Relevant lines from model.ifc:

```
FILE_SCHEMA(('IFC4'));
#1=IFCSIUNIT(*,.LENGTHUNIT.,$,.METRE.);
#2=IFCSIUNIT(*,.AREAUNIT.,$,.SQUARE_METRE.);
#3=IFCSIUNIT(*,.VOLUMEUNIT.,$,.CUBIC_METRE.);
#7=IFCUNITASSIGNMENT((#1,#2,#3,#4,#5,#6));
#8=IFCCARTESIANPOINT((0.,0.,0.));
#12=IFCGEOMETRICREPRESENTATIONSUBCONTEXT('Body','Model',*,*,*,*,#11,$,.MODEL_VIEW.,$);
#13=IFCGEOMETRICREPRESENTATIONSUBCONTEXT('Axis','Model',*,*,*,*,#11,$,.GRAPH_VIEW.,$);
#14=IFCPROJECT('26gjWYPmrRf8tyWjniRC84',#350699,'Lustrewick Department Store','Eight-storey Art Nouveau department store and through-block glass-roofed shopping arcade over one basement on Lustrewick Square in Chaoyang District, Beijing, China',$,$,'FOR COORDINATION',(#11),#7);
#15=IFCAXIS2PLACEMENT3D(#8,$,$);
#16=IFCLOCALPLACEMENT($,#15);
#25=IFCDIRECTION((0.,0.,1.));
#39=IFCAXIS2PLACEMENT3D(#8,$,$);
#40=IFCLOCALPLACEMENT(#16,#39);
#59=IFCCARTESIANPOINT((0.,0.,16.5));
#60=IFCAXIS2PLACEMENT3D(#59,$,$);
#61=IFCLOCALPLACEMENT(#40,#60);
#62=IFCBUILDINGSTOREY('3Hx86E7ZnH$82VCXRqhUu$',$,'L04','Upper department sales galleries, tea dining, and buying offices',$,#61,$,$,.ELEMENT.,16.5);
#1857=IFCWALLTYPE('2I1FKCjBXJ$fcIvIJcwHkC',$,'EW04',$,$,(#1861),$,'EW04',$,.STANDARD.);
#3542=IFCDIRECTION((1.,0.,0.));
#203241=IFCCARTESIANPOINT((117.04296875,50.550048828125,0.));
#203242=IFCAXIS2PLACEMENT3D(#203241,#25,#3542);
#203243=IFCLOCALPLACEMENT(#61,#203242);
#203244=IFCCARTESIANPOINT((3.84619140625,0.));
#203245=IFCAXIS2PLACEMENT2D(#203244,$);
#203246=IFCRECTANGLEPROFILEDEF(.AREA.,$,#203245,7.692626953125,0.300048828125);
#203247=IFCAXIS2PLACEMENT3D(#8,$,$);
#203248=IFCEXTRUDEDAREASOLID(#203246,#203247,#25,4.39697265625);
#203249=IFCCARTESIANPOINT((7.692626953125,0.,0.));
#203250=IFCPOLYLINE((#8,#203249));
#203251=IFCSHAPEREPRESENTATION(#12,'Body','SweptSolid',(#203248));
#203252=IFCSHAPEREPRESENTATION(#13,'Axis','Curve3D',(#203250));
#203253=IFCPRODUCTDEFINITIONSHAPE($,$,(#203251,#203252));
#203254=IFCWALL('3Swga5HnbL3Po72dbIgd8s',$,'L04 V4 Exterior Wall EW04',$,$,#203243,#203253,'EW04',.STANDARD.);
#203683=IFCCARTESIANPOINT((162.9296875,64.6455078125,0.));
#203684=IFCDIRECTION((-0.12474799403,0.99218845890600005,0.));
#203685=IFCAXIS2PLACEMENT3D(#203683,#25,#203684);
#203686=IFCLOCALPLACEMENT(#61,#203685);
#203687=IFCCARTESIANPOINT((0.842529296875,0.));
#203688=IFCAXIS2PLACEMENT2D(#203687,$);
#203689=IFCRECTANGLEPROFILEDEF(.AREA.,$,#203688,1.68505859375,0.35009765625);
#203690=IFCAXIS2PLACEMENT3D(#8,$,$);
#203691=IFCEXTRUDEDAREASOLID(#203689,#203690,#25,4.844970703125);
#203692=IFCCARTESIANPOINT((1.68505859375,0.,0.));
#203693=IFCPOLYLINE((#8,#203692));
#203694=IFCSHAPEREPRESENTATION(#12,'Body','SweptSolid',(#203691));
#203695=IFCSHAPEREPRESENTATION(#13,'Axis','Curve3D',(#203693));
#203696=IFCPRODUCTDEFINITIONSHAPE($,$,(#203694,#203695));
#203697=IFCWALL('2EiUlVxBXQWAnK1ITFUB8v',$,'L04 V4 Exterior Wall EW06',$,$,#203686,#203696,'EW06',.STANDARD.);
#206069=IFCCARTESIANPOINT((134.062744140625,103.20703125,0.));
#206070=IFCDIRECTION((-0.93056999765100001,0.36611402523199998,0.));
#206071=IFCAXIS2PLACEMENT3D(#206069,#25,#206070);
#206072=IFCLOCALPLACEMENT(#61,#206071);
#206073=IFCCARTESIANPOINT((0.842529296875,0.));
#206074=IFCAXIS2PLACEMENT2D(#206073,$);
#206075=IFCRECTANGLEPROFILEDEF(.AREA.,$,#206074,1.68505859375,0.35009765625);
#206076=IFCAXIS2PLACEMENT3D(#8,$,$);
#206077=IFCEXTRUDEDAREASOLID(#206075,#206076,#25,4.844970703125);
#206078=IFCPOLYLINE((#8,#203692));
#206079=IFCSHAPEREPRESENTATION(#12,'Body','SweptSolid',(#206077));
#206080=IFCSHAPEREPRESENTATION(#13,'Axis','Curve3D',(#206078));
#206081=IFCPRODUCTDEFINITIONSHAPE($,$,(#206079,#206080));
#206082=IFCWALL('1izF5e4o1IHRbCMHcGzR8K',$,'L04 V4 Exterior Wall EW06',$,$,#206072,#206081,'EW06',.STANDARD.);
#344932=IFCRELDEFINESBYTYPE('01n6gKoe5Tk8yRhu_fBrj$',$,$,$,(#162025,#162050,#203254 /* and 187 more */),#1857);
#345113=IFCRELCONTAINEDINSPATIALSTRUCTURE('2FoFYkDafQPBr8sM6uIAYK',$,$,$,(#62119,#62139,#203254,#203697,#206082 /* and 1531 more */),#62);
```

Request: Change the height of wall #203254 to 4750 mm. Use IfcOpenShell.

```python
import ifcopenshell
import ifcopenshell.geom
import ifcopenshell.util.representation
import ifcopenshell.util.shape
import ifcopenshell.util.unit

model = ifcopenshell.open("model.ifc")
unit_scale = ifcopenshell.util.unit.calculate_unit_scale(model)
settings = ifcopenshell.geom.settings()


def volume(element):
    """Net volume in cubic metres, openings subtracted."""
    shape = ifcopenshell.geom.create_shape(settings, element)
    return ifcopenshell.util.shape.get_volume(shape.geometry)


wall = model.by_guid("3Swga5HnbL3Po72dbIgd8s")
before = volume(wall)

body = ifcopenshell.util.representation.get_representation(wall, "Model", "Body")
solid = body.Items[0]
old_height = solid.Depth
solid.Depth = 4.75 / unit_scale
after = volume(wall)

print(f"height {old_height:g} -> {solid.Depth:g}, volume {before:.3f} -> {after:.3f} m3")

model.write("model_updated.ifc")
```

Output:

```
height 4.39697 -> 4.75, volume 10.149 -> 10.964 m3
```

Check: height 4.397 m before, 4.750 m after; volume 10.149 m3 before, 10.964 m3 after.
